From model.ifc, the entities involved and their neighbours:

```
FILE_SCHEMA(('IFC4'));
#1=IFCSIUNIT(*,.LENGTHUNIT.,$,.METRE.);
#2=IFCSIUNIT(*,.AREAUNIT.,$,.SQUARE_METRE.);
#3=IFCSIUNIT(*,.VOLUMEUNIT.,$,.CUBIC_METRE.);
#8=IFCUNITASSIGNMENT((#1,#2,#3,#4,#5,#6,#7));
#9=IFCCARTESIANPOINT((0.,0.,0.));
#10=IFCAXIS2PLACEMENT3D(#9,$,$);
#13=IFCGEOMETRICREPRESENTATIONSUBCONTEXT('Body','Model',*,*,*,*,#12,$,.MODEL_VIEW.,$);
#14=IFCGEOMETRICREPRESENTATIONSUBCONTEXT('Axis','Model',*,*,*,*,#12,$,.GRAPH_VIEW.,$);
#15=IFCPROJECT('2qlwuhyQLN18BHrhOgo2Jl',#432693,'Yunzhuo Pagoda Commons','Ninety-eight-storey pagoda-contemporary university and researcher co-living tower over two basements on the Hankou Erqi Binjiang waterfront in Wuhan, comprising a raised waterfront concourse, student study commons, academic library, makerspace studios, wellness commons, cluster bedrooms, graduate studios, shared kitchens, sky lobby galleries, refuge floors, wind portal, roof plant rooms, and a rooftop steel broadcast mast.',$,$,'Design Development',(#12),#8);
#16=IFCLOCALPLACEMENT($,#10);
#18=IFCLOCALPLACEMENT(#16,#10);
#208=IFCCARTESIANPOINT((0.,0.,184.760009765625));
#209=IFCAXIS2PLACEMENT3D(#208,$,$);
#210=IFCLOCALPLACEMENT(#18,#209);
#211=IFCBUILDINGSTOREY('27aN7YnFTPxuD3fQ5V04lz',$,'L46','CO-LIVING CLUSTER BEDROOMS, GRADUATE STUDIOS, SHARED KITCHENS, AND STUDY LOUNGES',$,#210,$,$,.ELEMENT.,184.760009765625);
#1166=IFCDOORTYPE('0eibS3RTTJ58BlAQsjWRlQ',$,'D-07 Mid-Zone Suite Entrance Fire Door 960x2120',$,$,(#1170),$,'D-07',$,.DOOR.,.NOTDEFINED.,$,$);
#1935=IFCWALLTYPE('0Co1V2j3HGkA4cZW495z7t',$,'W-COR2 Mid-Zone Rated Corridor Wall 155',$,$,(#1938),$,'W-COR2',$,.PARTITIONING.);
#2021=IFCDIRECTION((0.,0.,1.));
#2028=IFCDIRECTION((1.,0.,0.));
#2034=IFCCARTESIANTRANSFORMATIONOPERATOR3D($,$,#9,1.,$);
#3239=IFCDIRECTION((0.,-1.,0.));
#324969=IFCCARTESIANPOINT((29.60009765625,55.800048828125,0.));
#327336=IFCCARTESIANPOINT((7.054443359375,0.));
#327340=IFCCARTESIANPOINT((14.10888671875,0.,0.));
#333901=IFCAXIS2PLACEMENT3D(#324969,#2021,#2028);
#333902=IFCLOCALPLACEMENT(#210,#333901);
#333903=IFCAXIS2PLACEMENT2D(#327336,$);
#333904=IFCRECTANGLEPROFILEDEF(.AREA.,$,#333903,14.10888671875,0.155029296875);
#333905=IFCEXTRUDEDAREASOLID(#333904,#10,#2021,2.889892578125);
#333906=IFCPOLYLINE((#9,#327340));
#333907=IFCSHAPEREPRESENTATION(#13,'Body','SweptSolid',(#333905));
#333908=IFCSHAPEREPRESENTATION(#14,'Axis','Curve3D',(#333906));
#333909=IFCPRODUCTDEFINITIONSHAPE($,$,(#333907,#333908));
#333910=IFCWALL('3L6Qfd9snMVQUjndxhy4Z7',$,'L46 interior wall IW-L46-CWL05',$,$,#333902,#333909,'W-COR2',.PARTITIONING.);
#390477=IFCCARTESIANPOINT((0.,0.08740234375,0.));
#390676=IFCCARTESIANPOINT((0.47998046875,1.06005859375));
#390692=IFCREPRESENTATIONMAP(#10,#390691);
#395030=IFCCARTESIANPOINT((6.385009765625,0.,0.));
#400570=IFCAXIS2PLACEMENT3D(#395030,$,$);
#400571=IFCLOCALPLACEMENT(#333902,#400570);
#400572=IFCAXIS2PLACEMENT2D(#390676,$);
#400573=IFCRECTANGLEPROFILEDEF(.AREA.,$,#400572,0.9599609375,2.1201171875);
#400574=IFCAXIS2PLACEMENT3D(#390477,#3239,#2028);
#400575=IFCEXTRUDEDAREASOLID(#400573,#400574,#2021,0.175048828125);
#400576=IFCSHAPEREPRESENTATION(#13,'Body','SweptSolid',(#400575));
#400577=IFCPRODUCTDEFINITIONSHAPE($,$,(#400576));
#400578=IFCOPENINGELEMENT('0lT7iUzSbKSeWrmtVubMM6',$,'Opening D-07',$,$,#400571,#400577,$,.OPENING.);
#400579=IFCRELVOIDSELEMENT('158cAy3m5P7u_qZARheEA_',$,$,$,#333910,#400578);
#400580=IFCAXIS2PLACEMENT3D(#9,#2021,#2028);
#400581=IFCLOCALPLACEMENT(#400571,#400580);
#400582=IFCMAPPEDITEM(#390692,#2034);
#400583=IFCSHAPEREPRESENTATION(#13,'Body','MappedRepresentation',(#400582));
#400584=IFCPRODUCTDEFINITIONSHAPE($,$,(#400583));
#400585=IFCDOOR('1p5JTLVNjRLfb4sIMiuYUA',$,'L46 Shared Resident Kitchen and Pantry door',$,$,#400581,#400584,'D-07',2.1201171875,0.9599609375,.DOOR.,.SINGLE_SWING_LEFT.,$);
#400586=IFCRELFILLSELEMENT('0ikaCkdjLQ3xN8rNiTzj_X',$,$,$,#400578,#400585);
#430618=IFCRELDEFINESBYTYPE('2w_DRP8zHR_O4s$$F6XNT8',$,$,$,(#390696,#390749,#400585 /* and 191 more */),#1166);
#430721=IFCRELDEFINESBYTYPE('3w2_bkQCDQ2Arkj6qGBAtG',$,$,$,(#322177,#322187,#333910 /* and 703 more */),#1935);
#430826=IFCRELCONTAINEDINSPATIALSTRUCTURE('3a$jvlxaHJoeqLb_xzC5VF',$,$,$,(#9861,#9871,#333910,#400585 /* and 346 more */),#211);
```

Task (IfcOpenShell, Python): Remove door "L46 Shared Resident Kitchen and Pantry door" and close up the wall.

```python
import ifcopenshell
import ifcopenshell.api.feature
import ifcopenshell.api.root
import ifcopenshell.geom
import ifcopenshell.util.shape

model = ifcopenshell.open("model.ifc")
settings = ifcopenshell.geom.settings()


def volume(element):
    """Net volume in cubic metres, openings subtracted."""
    shape = ifcopenshell.geom.create_shape(settings, element)
    return ifcopenshell.util.shape.get_volume(shape.geometry)


door = model.by_guid("1p5JTLVNjRLfb4sIMiuYUA")
opening = door.FillsVoids[0].RelatingOpeningElement
wall = opening.VoidsElements[0].RelatingBuildingElement
before = volume(wall)

ifcopenshell.api.root.remove_product(model, product=door)
ifcopenshell.api.feature.remove_feature(model, feature=opening)

after = volume(wall)

print(f"wall volume {before:.3f} -> {after:.3f} m3")

model.write("model_v2.ifc")
```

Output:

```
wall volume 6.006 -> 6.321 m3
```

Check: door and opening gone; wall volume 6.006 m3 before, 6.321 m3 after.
